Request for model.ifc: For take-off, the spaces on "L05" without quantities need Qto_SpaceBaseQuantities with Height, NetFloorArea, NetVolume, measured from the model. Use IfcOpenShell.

First a look at what the model holds.

```python
import ifcopenshell
import ifcopenshell.util.element
import ifcopenshell.util.unit

model = ifcopenshell.open("model.ifc")
print(model.schema)
for unit_type in ("LENGTHUNIT", "AREAUNIT", "VOLUMEUNIT"):
    print(unit_type, ifcopenshell.util.unit.calculate_unit_scale(model, unit_type))
storey = next(s for s in model.by_type("IfcBuildingStorey") if s.Name == "L05")
spaces = [e for e in ifcopenshell.util.element.get_decomposition(storey) if e.is_a("IfcSpace")]
for e in sorted(spaces, key=lambda e: e.id()):
    print(e.id(), e.is_a(), e.Name, list(ifcopenshell.util.element.get_psets(e, qtos_only=True)), sep=" | ")
```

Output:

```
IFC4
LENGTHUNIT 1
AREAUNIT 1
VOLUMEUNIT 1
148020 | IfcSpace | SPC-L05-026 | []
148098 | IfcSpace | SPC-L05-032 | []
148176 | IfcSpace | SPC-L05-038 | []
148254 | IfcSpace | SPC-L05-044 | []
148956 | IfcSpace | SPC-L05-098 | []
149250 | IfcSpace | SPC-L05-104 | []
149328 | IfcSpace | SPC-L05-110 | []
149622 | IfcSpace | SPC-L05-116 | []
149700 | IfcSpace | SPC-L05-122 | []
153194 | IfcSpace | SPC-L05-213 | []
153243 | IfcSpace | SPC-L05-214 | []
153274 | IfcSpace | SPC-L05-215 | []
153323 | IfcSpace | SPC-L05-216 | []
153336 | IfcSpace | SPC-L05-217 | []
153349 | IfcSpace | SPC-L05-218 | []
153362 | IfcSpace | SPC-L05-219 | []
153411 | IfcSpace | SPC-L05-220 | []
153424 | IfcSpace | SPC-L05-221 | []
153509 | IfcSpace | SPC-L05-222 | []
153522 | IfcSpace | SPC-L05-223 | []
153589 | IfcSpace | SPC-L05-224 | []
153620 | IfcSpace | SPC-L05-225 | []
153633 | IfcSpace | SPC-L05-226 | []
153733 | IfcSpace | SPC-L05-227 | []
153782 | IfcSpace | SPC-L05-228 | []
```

```python
import ifcopenshell
import ifcopenshell.api.pset
import ifcopenshell.geom
import ifcopenshell.util.element
import ifcopenshell.util.shape
import ifcopenshell.util.unit

model = ifcopenshell.open("model.ifc")
unit_scale = ifcopenshell.util.unit.calculate_unit_scale(model)
area_scale = ifcopenshell.util.unit.calculate_unit_scale(model, "AREAUNIT")
volume_scale = ifcopenshell.util.unit.calculate_unit_scale(model, "VOLUMEUNIT")
settings = ifcopenshell.geom.settings()

storey = next(s for s in model.by_type("IfcBuildingStorey") if s.Name == "L05")
spaces = [e for e in ifcopenshell.util.element.get_decomposition(storey) if e.is_a("IfcSpace")]

for e in sorted(spaces, key=lambda e: e.id()):
    if ifcopenshell.util.element.get_psets(e, qtos_only=True, should_inherit=False):
        continue
    # Geometry comes back in metres, in the element's own axes.
    shape = ifcopenshell.geom.create_shape(settings, e)
    values = {
        "Height": ifcopenshell.util.shape.get_z(shape.geometry) / unit_scale,
        "NetFloorArea": ifcopenshell.util.shape.get_footprint_area(shape.geometry) / area_scale,
        "NetVolume": ifcopenshell.util.shape.get_volume(shape.geometry) / volume_scale,
    }
    qto = ifcopenshell.api.pset.add_qto(model, product=e, name="Qto_SpaceBaseQuantities")
    ifcopenshell.api.pset.edit_qto(model, qto=qto, properties=values)
    print(e.id(), {k: round(v, 3) for k, v in values.items()})

model.write("model_edited.ifc")
```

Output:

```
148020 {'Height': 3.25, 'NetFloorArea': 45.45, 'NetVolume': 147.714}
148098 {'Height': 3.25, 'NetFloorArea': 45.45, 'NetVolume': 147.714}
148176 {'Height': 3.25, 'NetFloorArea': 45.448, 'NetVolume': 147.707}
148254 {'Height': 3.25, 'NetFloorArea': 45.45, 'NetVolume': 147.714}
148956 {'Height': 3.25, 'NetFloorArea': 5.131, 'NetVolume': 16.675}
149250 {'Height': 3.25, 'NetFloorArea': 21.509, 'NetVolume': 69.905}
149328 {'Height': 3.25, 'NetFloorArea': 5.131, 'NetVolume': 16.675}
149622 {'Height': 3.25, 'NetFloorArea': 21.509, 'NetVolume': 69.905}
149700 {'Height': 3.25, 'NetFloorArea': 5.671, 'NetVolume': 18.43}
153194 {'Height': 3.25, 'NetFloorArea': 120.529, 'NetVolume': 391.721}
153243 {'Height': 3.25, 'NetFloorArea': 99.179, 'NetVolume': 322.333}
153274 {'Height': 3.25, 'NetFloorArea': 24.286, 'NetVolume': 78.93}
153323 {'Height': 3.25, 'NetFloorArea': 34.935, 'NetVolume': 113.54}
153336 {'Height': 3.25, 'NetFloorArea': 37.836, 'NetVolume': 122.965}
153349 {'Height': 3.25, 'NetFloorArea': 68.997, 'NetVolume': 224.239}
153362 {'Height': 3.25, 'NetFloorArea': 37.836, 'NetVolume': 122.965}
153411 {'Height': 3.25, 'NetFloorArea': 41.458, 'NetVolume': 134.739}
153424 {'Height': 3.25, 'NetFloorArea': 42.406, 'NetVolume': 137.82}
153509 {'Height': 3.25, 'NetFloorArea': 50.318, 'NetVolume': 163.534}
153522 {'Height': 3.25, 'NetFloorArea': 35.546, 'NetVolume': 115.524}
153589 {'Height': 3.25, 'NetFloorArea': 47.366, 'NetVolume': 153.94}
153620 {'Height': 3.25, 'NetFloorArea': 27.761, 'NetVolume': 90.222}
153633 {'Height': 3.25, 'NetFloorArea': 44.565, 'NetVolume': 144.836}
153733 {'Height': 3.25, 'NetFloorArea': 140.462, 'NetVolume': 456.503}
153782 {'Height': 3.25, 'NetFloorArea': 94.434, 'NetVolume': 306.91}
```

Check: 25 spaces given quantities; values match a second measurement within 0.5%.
